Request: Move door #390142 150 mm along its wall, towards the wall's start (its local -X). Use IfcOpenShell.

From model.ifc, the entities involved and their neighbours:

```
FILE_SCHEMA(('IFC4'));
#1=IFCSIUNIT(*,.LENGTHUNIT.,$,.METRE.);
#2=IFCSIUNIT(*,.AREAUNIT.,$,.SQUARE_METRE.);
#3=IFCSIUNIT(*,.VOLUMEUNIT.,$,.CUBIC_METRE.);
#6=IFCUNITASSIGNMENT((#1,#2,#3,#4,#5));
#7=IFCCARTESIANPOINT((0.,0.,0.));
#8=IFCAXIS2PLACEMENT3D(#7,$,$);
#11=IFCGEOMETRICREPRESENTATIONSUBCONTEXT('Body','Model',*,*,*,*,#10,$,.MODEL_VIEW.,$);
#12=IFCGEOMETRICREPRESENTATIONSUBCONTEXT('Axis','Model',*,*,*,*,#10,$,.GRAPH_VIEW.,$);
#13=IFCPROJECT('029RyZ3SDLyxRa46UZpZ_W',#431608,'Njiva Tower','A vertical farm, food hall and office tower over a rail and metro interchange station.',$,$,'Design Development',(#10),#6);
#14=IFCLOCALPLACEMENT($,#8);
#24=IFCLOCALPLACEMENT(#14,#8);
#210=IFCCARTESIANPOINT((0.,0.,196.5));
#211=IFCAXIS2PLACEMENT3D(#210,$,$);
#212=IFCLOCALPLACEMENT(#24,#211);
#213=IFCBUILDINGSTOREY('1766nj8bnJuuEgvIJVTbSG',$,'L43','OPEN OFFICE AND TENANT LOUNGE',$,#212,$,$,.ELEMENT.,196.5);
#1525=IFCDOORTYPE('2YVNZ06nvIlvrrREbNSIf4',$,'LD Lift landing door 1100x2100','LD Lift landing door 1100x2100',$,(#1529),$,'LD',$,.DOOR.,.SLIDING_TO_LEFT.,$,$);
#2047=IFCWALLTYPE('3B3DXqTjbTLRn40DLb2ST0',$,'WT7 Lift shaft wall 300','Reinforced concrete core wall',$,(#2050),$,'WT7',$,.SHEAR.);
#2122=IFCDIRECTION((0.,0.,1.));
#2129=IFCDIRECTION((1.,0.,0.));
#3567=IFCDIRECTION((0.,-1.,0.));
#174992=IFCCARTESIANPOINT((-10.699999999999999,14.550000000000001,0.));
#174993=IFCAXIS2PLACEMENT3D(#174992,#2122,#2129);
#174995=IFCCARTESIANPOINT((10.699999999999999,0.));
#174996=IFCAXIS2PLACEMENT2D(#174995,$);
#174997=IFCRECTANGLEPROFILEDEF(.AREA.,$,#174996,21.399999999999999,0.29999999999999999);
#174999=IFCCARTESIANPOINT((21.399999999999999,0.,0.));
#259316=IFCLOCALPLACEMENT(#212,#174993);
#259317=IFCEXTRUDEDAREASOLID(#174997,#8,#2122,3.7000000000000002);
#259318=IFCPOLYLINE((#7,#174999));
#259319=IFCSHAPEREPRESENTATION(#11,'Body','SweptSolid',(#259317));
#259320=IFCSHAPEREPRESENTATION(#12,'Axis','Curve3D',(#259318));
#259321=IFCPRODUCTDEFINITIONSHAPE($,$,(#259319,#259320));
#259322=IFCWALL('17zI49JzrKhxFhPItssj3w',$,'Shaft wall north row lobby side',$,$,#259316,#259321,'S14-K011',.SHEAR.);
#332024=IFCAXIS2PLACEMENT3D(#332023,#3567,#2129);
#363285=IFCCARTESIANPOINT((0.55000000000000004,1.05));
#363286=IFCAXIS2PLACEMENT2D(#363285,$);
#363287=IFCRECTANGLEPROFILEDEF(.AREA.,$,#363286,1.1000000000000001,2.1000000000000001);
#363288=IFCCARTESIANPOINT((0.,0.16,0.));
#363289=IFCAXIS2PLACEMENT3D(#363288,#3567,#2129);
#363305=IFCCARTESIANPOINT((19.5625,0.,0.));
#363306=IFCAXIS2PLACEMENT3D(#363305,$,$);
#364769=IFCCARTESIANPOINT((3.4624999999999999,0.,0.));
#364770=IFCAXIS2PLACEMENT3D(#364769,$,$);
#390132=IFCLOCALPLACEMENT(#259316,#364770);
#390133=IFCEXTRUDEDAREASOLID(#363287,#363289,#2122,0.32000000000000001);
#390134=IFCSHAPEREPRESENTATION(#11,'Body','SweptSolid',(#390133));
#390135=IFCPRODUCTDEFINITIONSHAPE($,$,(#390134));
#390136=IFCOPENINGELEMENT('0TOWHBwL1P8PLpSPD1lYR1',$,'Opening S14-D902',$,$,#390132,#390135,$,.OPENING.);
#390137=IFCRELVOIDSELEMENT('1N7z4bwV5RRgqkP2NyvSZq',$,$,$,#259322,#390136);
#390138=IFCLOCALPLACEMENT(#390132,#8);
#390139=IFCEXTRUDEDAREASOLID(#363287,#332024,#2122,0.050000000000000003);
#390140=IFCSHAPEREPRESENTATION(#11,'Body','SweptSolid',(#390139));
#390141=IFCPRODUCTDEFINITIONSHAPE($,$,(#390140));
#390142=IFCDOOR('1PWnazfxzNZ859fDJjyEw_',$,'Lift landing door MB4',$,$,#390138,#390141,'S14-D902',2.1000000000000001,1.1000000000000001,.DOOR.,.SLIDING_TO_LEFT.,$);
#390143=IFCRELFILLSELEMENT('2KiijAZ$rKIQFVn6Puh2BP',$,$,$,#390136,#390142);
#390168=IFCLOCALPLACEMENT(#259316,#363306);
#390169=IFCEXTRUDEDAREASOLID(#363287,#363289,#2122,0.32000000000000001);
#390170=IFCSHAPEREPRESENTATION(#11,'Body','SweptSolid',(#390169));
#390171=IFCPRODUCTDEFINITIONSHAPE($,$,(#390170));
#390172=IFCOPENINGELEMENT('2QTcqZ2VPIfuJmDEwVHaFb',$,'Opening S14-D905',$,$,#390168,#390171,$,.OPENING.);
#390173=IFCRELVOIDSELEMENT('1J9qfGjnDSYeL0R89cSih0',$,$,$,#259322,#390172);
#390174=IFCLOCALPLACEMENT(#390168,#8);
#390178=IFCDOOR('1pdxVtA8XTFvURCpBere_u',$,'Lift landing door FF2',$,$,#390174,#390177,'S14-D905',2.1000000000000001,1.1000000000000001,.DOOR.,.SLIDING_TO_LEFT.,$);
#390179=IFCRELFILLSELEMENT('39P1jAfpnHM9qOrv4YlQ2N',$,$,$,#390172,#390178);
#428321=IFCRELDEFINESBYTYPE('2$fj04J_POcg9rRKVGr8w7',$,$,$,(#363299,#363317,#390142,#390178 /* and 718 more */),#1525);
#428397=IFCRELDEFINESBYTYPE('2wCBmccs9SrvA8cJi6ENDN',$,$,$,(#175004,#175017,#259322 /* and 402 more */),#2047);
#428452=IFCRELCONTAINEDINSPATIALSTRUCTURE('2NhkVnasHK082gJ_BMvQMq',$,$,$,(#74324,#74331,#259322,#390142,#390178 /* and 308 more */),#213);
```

```python
import ifcopenshell
import ifcopenshell.api.geometry
import ifcopenshell.util.placement
import ifcopenshell.util.unit

model = ifcopenshell.open("model.ifc")
unit_scale = ifcopenshell.util.unit.calculate_unit_scale(model)

door = model.by_id(390142)
opening = door.FillsVoids[0].RelatingOpeningElement
wall = opening.VoidsElements[0].RelatingBuildingElement

wall_matrix = ifcopenshell.util.placement.get_local_placement(wall.ObjectPlacement)
shift = wall_matrix[:3, 0] * -0.15 / unit_scale
before = ifcopenshell.util.placement.get_local_placement(door.ObjectPlacement)[:3, 3].copy()

# The door is placed relative to its opening, so it follows when the opening moves.
matrix = ifcopenshell.util.placement.get_local_placement(opening.ObjectPlacement)
matrix[:3, 3] += shift
ifcopenshell.api.geometry.edit_object_placement(
    model, product=opening, matrix=matrix, is_si=False, should_transform_children=True
)

after = ifcopenshell.util.placement.get_local_placement(door.ObjectPlacement)[:3, 3]
print("door moved by", (after - before).round(3) + 0.0)

model.write("model-out.ifc")
```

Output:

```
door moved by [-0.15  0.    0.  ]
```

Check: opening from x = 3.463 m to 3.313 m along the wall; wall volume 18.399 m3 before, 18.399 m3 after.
